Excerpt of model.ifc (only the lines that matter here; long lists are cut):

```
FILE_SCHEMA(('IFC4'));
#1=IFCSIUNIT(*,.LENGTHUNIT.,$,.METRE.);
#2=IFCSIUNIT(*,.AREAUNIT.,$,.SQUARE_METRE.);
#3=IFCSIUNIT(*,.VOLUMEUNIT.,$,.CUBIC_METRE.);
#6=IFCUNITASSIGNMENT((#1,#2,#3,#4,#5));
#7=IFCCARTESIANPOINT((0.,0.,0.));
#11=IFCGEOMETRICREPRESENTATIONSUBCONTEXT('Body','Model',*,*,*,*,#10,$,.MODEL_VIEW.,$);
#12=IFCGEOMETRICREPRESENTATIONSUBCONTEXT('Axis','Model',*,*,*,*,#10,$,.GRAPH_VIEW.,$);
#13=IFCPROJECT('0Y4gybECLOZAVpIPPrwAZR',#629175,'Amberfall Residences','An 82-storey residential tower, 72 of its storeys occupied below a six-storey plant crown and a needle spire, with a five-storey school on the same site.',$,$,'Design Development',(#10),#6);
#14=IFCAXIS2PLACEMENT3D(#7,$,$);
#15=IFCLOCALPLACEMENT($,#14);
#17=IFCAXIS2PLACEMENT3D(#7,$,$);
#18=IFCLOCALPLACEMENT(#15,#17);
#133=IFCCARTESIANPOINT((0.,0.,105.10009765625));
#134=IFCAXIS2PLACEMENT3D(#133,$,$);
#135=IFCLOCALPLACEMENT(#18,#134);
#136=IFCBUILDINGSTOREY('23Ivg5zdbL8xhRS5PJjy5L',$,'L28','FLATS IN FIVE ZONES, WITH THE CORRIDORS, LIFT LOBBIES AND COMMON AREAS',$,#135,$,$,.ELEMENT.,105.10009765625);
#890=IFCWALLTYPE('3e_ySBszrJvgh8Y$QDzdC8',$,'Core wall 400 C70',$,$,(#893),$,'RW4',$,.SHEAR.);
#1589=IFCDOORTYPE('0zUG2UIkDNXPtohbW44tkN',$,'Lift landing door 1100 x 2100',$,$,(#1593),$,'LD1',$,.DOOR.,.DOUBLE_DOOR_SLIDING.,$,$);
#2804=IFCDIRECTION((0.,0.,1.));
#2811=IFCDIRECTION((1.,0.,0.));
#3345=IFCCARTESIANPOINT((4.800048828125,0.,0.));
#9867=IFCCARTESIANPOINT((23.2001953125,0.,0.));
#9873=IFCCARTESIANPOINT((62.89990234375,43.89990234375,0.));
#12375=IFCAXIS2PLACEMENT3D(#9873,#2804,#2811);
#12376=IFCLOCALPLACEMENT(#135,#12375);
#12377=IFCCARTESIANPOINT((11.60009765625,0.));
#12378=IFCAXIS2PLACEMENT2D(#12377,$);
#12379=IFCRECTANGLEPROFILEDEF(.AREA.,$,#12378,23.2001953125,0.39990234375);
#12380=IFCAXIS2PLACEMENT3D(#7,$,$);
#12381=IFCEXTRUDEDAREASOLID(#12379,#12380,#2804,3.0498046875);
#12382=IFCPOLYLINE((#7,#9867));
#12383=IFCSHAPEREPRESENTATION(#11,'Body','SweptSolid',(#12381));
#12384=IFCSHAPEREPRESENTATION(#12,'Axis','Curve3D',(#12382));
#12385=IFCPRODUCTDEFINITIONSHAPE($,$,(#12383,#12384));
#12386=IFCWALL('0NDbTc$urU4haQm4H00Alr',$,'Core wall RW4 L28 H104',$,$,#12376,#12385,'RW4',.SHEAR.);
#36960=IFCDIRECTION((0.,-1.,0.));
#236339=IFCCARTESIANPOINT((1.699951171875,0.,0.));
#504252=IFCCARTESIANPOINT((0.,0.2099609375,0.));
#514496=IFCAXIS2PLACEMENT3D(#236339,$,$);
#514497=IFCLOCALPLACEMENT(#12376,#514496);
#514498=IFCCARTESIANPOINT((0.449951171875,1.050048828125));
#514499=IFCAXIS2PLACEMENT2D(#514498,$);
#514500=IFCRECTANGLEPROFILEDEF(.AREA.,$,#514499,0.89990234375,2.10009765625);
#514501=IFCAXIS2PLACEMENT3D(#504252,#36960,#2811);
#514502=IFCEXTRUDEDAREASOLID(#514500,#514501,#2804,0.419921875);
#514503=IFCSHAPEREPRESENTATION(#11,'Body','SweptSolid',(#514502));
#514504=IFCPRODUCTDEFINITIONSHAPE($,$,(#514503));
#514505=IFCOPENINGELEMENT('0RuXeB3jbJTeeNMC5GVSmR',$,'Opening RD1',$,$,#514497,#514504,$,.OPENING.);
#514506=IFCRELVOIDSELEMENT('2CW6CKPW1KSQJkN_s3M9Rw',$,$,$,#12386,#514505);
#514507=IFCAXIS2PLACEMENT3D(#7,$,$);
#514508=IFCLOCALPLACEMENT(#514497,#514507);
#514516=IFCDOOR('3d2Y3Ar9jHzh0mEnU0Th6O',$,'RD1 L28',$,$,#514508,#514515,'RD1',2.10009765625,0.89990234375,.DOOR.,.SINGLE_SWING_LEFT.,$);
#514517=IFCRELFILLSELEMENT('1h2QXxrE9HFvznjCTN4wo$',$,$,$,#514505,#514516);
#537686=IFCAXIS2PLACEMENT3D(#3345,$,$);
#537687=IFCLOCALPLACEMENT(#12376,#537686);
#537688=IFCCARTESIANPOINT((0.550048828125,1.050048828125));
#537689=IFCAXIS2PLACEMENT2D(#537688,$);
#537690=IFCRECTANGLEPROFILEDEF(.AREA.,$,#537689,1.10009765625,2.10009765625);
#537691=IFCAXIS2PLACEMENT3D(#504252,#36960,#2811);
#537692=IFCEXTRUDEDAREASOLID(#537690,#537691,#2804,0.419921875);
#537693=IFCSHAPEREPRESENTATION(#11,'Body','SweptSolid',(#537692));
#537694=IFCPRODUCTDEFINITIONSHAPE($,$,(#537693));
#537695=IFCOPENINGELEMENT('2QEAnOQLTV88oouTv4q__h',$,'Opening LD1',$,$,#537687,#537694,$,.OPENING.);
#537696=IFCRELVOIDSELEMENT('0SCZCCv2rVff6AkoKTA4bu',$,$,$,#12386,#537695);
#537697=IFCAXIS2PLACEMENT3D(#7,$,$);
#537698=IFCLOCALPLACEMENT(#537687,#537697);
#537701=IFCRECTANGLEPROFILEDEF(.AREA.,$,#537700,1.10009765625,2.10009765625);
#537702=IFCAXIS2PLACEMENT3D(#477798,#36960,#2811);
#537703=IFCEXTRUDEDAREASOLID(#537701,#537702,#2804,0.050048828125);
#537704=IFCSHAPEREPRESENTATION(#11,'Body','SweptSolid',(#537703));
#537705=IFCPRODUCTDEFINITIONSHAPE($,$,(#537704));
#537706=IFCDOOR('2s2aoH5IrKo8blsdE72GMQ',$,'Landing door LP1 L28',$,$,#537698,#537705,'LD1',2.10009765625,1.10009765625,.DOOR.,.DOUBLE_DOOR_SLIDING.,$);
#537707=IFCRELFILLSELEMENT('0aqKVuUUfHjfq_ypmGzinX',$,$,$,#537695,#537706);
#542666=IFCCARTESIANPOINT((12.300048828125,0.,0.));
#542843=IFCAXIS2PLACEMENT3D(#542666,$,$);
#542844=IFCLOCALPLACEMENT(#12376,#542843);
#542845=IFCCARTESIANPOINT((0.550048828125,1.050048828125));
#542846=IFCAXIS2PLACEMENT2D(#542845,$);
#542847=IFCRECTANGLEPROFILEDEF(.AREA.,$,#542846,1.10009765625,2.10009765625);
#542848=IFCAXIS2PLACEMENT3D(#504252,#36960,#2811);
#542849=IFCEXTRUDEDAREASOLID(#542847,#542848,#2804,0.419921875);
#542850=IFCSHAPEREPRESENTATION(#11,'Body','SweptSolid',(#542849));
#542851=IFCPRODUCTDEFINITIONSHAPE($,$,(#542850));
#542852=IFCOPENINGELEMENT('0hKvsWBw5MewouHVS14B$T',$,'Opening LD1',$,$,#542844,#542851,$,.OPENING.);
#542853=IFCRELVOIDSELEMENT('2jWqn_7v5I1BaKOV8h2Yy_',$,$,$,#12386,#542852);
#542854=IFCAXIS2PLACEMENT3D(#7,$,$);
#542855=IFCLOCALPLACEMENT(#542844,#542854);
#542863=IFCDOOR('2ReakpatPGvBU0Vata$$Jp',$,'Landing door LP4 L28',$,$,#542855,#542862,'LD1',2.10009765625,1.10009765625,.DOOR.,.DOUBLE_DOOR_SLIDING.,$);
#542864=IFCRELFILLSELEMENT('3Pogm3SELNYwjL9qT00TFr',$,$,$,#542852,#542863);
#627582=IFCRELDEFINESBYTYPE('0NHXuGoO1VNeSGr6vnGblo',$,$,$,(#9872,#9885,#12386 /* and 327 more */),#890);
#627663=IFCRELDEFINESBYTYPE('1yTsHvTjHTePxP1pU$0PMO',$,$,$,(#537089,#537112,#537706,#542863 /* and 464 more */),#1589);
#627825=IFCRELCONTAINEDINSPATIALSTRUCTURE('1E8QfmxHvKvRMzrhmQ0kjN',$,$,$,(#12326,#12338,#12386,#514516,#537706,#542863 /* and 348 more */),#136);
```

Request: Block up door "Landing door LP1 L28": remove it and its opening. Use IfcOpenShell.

```python
import ifcopenshell
import ifcopenshell.api.feature
import ifcopenshell.api.root
import ifcopenshell.geom
import ifcopenshell.util.shape

model = ifcopenshell.open("model.ifc")
settings = ifcopenshell.geom.settings()


def volume(element):
    """Net volume in cubic metres, openings subtracted."""
    shape = ifcopenshell.geom.create_shape(settings, element)
    return ifcopenshell.util.shape.get_volume(shape.geometry)


door = model.by_guid("2s2aoH5IrKo8blsdE72GMQ")
opening = door.FillsVoids[0].RelatingOpeningElement
wall = opening.VoidsElements[0].RelatingBuildingElement
before = volume(wall)

ifcopenshell.api.root.remove_product(model, product=door)
ifcopenshell.api.feature.remove_feature(model, feature=opening)

after = volume(wall)

print(f"wall volume {before:.3f} -> {after:.3f} m3")

model.write("model_edited.ifc")
```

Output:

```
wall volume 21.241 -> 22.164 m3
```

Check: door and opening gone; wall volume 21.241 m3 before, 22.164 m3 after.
